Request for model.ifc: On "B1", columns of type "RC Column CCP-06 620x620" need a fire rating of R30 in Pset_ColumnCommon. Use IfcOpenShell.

First a look at what the model holds.

```python
import ifcopenshell
import ifcopenshell.util.element

model = ifcopenshell.open("model.ifc")
print(model.schema)
storey = next(s for s in model.by_type("IfcBuildingStorey") if s.Name == "B1")
columns = [e for e in ifcopenshell.util.element.get_decomposition(storey) if e.is_a("IfcColumn")]
seen = {}
for e in columns:
    element_type = ifcopenshell.util.element.get_type(e)
    key = (element_type.Name if element_type != e and element_type else None, ifcopenshell.util.element.get_pset(e, "Pset_ColumnCommon", "FireRating"))
    seen[key] = seen.get(key, 0) + 1
for (name, value), count in sorted(seen.items(), key=str):
    print(count, "x", name, "|", value)
```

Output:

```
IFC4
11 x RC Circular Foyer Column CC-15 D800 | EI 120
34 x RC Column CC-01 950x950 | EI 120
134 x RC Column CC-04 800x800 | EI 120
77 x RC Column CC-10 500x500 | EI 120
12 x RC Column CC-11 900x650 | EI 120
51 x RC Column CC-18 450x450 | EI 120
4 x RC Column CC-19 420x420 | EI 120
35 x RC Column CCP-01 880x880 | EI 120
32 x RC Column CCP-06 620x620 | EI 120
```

```python
import ifcopenshell
import ifcopenshell.api.pset
import ifcopenshell.util.element

model = ifcopenshell.open("model.ifc")

storey = next(s for s in model.by_type("IfcBuildingStorey") if s.Name == "B1")
columns = [e for e in ifcopenshell.util.element.get_decomposition(storey) if e.is_a("IfcColumn")]

count = 0
for e in columns:
    element_type = ifcopenshell.util.element.get_type(e)
    if element_type in (None, e) or element_type.Name != "RC Column CCP-06 620x620":
        continue
    # add_pset returns the element's existing set when there is one.
    pset = ifcopenshell.api.pset.add_pset(model, product=e, name="Pset_ColumnCommon")
    ifcopenshell.api.pset.edit_pset(model, pset=pset, properties={"FireRating": "R30"})
    count += 1

print(count, "columns updated")

model.write("model_updated.ifc")
```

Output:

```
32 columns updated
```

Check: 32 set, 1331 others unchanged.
